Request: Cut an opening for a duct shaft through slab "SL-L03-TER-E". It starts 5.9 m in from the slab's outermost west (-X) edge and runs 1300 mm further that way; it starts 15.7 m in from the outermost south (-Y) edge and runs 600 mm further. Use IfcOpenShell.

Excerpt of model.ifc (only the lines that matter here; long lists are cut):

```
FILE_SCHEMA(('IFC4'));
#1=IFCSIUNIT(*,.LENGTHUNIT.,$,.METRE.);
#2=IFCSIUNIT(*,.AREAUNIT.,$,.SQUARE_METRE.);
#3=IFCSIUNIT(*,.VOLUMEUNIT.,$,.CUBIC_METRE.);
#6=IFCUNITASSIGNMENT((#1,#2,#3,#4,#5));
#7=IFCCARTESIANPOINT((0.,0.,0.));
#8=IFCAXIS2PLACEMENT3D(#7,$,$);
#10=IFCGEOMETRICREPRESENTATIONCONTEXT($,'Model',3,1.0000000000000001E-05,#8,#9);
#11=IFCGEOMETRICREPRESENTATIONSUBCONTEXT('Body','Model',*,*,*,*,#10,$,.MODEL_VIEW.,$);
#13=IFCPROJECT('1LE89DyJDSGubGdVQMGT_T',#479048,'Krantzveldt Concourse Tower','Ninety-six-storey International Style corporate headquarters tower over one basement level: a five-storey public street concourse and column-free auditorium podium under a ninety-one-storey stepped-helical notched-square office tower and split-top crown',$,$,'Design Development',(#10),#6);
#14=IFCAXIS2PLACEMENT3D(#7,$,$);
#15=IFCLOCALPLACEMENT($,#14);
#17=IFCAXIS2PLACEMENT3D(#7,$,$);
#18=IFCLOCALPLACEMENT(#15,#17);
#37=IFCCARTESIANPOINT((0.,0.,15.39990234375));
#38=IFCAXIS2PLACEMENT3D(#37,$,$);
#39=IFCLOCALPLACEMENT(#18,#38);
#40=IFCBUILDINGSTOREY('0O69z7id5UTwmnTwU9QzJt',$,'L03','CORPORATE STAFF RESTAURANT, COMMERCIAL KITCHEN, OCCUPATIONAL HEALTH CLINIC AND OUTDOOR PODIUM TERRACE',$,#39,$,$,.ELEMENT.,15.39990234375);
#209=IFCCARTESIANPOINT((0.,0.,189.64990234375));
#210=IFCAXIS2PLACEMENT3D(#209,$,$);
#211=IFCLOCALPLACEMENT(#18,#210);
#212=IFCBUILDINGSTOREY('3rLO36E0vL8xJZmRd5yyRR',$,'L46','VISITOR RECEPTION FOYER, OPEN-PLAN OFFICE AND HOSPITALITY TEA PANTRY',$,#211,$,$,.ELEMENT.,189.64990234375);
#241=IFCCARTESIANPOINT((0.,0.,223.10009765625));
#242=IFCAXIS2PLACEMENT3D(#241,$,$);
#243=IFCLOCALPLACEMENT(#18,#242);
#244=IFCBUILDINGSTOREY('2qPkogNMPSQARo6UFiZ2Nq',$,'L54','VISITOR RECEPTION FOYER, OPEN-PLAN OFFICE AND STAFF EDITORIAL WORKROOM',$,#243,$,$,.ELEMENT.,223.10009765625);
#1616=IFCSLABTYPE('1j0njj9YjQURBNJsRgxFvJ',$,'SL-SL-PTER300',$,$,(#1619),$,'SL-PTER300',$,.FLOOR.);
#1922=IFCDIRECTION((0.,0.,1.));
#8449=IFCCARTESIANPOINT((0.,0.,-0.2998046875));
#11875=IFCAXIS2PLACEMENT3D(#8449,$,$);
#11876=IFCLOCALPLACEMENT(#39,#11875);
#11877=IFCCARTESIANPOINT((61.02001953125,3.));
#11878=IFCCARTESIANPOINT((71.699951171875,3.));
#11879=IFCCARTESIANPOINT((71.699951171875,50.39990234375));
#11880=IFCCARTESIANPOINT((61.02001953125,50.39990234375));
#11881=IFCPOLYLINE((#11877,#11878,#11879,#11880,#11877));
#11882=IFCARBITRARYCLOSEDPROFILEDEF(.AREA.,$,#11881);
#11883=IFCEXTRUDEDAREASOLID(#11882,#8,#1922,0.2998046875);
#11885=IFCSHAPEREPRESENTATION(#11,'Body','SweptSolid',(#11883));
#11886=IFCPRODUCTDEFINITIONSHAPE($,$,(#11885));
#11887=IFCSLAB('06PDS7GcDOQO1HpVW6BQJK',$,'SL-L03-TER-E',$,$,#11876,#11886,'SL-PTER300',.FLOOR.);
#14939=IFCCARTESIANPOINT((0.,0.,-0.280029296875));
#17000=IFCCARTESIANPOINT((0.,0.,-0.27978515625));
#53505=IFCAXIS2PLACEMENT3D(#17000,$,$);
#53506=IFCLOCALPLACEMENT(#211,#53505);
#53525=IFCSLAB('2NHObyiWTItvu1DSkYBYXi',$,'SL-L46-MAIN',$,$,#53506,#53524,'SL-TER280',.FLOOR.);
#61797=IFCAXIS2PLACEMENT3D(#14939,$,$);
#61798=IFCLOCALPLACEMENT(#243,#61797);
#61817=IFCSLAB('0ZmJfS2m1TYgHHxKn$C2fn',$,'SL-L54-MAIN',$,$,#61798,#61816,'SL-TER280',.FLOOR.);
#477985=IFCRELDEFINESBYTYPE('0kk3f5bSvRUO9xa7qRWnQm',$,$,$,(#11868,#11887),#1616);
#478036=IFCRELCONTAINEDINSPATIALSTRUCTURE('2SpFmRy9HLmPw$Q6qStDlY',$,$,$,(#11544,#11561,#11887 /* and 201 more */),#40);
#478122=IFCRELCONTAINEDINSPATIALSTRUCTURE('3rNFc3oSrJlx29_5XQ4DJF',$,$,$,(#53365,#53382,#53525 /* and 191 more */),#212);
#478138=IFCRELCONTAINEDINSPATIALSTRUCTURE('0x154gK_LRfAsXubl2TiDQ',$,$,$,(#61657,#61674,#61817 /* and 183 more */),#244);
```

```python
import numpy as np
import ifcopenshell
import ifcopenshell.api.feature
import ifcopenshell.api.geometry
import ifcopenshell.api.root
import ifcopenshell.geom
import ifcopenshell.util.placement
import ifcopenshell.util.representation
import ifcopenshell.util.shape
import ifcopenshell.util.unit

model = ifcopenshell.open("model.ifc")
unit_scale = ifcopenshell.util.unit.calculate_unit_scale(model)
settings = ifcopenshell.geom.settings()


def volume(element):
    """Net volume in cubic metres, openings subtracted."""
    shape = ifcopenshell.geom.create_shape(settings, element)
    return ifcopenshell.util.shape.get_volume(shape.geometry)


slab = model.by_guid("06PDS7GcDOQO1HpVW6BQJK")
before = volume(slab)

# Extent in the slab's own axes, in metres. The edges named are its -X and -Y sides.
slab_shape = ifcopenshell.geom.create_shape(settings, slab)
vertices = ifcopenshell.util.shape.get_vertices(slab_shape.geometry)
x_min, y_min, bottom = vertices.min(axis=0)
top = vertices[:, 2].max()

opening = ifcopenshell.api.root.create_entity(model, ifc_class="IfcOpeningElement", name="Duct shaft opening", predefined_type="OPENING")
context = ifcopenshell.util.representation.get_context(model, "Model", "Body", "MODEL_VIEW")
width, depth = 1.3, 0.6
outline = [(0.0, 0.0), (width, 0.0), (width, depth), (0.0, depth), (0.0, 0.0)]
# Overshoot both faces by 50 mm so the cut is clean.
shape = ifcopenshell.api.geometry.add_slab_representation(
    model, context=context, depth=top - bottom + 0.1, polyline=outline
)
ifcopenshell.api.geometry.assign_representation(model, product=opening, representation=shape)

matrix = ifcopenshell.util.placement.get_local_placement(slab.ObjectPlacement)
matrix[:, 3] = matrix @ np.append(np.array([x_min + 5.9, y_min + 15.7, bottom - 0.05]) / unit_scale, 1.0)
ifcopenshell.api.geometry.edit_object_placement(model, product=opening, matrix=matrix, is_si=False)
ifcopenshell.api.feature.add_feature(model, feature=opening, element=slab)

after = volume(slab)

print(f"slab volume {before:.3f} -> {after:.3f} m3")

model.write("model_edited.ifc")
```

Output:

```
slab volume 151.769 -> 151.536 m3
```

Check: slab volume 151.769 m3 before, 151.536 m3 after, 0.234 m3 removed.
